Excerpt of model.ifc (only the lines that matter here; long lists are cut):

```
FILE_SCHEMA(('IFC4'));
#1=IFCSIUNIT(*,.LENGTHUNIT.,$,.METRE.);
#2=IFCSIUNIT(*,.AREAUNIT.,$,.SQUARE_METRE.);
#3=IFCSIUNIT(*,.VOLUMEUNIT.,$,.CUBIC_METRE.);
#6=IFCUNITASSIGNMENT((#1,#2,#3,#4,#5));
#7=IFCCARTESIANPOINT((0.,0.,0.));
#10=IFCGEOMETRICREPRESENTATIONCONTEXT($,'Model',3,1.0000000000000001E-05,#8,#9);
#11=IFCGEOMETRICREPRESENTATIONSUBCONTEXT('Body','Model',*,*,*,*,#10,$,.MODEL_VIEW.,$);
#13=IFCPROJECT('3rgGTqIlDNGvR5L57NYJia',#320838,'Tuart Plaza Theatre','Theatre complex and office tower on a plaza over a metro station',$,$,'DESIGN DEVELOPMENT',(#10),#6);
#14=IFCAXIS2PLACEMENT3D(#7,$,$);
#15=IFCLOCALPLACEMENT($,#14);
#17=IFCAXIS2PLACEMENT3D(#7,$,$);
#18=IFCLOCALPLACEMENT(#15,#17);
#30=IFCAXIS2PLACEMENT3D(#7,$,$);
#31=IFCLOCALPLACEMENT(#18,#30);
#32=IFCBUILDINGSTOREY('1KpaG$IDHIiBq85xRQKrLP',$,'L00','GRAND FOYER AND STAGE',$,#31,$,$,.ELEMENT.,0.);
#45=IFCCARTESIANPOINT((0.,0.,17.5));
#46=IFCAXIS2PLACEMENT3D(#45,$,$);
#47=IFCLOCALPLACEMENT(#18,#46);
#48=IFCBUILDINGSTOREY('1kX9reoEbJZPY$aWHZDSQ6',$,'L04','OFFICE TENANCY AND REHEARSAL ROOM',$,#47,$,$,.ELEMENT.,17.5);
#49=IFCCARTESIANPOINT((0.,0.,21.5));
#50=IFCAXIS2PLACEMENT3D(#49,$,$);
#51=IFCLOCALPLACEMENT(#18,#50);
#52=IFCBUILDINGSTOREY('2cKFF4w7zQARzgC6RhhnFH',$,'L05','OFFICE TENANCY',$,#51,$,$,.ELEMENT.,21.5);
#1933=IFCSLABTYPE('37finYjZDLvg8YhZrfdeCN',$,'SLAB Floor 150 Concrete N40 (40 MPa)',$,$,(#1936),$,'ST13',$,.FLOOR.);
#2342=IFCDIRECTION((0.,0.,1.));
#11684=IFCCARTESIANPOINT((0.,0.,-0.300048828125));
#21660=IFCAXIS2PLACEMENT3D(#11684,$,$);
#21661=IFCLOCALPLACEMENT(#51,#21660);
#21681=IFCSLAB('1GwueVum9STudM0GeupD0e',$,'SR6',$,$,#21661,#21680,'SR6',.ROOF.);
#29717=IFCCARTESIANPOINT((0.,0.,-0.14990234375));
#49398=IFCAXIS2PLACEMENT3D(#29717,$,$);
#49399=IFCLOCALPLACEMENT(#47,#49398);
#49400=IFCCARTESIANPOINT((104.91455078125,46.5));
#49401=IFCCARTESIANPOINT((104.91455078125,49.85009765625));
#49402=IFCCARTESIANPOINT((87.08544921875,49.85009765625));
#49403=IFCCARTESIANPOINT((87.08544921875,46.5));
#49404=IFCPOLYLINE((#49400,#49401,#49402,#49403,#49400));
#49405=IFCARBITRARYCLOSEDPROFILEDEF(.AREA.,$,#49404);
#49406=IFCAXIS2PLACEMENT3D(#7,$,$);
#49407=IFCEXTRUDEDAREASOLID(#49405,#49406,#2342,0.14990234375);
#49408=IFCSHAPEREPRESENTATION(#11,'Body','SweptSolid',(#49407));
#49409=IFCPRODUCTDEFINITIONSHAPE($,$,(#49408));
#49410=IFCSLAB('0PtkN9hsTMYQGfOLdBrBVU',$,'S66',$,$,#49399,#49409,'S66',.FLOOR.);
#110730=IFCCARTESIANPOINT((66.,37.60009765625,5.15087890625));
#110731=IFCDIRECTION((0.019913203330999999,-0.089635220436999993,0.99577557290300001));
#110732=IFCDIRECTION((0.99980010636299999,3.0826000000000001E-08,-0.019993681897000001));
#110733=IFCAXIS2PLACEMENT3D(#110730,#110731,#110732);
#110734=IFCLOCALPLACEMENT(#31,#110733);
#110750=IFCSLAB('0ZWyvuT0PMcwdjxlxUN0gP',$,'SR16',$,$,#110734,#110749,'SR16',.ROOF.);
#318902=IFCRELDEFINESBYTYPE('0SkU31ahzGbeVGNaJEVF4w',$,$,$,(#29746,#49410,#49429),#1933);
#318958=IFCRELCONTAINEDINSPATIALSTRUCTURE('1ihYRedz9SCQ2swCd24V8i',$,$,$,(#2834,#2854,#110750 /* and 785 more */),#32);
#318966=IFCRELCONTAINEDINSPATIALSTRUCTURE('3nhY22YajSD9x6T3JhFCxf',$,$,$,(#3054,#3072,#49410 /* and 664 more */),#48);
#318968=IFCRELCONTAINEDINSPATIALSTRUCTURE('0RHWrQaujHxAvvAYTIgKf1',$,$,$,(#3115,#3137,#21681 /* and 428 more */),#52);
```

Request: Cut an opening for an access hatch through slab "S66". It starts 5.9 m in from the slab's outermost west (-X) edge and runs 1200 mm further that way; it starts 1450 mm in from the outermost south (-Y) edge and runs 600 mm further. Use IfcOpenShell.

```python
import numpy as np
import ifcopenshell
import ifcopenshell.api.feature
import ifcopenshell.api.geometry
import ifcopenshell.api.root
import ifcopenshell.geom
import ifcopenshell.util.placement
import ifcopenshell.util.representation
import ifcopenshell.util.shape
import ifcopenshell.util.unit

model = ifcopenshell.open("model.ifc")
unit_scale = ifcopenshell.util.unit.calculate_unit_scale(model)
settings = ifcopenshell.geom.settings()


def volume(element):
    """Net volume in cubic metres, openings subtracted."""
    shape = ifcopenshell.geom.create_shape(settings, element)
    return ifcopenshell.util.shape.get_volume(shape.geometry)


slab = model.by_id(49410)
before = volume(slab)

# Extent in the slab's own axes, in metres. The edges named are its -X and -Y sides.
slab_shape = ifcopenshell.geom.create_shape(settings, slab)
vertices = ifcopenshell.util.shape.get_vertices(slab_shape.geometry)
x_min, y_min, bottom = vertices.min(axis=0)
top = vertices[:, 2].max()

opening = ifcopenshell.api.root.create_entity(model, ifc_class="IfcOpeningElement", name="Access hatch opening", predefined_type="OPENING")
context = ifcopenshell.util.representation.get_context(model, "Model", "Body", "MODEL_VIEW")
width, depth = 1.2, 0.6
outline = [(0.0, 0.0), (width, 0.0), (width, depth), (0.0, depth), (0.0, 0.0)]
# Overshoot both faces by 50 mm so the cut is clean.
shape = ifcopenshell.api.geometry.add_slab_representation(
    model, context=context, depth=top - bottom + 0.1, polyline=outline
)
ifcopenshell.api.geometry.assign_representation(model, product=opening, representation=shape)

matrix = ifcopenshell.util.placement.get_local_placement(slab.ObjectPlacement)
matrix[:, 3] = matrix @ np.append(np.array([x_min + 5.9, y_min + 1.45, bottom - 0.05]) / unit_scale, 1.0)
ifcopenshell.api.geometry.edit_object_placement(model, product=opening, matrix=matrix, is_si=False)
ifcopenshell.api.feature.add_feature(model, feature=opening, element=slab)

after = volume(slab)

print(f"slab volume {before:.3f} -> {after:.3f} m3")

model.write("model_rev.ifc")
```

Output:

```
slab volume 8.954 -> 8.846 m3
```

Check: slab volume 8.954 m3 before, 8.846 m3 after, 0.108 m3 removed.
